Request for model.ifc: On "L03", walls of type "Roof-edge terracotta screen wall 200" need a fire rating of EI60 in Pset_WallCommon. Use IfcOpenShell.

First a look at what the model holds.

```python
import ifcopenshell
import ifcopenshell.util.element

model = ifcopenshell.open("model.ifc")
print(model.schema)
storey = next(s for s in model.by_type("IfcBuildingStorey") if s.Name == "L03")
walls = [e for e in ifcopenshell.util.element.get_decomposition(storey) if e.is_a("IfcWall")]
seen = {}
for e in walls:
    element_type = ifcopenshell.util.element.get_type(e)
    key = (element_type.Name if element_type != e and element_type else None, ifcopenshell.util.element.get_pset(e, "Pset_WallCommon", "FireRating"))
    seen[key] = seen.get(key, 0) + 1
for (name, value), count in sorted(seen.items(), key=str):
    print(count, "x", name, "|", value)
```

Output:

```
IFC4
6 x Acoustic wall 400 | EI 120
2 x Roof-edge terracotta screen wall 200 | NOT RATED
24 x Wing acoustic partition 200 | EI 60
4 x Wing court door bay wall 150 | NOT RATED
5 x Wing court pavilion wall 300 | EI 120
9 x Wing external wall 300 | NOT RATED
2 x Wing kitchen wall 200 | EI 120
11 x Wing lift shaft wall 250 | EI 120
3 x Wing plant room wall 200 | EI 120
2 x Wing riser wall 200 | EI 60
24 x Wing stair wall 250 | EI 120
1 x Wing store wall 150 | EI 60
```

```python
import ifcopenshell
import ifcopenshell.api.pset
import ifcopenshell.util.element

model = ifcopenshell.open("model.ifc")

storey = next(s for s in model.by_type("IfcBuildingStorey") if s.Name == "L03")
walls = [e for e in ifcopenshell.util.element.get_decomposition(storey) if e.is_a("IfcWall")]

count = 0
for e in walls:
    element_type = ifcopenshell.util.element.get_type(e)
    if element_type in (None, e) or element_type.Name != "Roof-edge terracotta screen wall 200":
        continue
    # add_pset returns the element's existing set when there is one.
    pset = ifcopenshell.api.pset.add_pset(model, product=e, name="Pset_WallCommon")
    ifcopenshell.api.pset.edit_pset(model, pset=pset, properties={"FireRating": "EI60"})
    count += 1

print(count, "walls updated")

model.write("model-out.ifc")
```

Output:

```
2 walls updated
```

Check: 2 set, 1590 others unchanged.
